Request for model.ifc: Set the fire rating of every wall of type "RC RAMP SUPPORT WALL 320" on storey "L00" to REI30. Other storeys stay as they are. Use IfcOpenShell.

First a look at what the model holds.

```python
import ifcopenshell
import ifcopenshell.util.element

model = ifcopenshell.open("model.ifc")
print(model.schema)
storey = next(s for s in model.by_type("IfcBuildingStorey") if s.Name == "L00")
walls = [e for e in ifcopenshell.util.element.get_decomposition(storey) if e.is_a("IfcWall")]
seen = {}
for e in walls:
    element_type = ifcopenshell.util.element.get_type(e)
    key = (element_type.Name if element_type != e and element_type else None, ifcopenshell.util.element.get_pset(e, "Pset_WallCommon", "FireRating"))
    seen[key] = seen.get(key, 0) + 1
for (name, value), count in sorted(seen.items(), key=str):
    print(count, "x", name, "|", value)
```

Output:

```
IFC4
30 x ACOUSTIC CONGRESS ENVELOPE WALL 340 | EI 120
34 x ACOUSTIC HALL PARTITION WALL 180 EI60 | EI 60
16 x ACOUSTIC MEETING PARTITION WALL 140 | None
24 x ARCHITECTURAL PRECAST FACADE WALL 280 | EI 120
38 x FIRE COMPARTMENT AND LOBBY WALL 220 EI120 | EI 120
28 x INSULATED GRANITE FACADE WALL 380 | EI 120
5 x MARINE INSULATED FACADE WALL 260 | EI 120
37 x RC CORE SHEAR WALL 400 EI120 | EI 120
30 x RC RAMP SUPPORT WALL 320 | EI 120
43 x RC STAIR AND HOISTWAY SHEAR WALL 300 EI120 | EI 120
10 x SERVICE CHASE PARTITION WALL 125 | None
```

```python
import ifcopenshell
import ifcopenshell.api.pset
import ifcopenshell.util.element

model = ifcopenshell.open("model.ifc")

storey = next(s for s in model.by_type("IfcBuildingStorey") if s.Name == "L00")
walls = [e for e in ifcopenshell.util.element.get_decomposition(storey) if e.is_a("IfcWall")]

count = 0
for e in walls:
    element_type = ifcopenshell.util.element.get_type(e)
    if element_type in (None, e) or element_type.Name != "RC RAMP SUPPORT WALL 320":
        continue
    # add_pset returns the element's existing set when there is one.
    pset = ifcopenshell.api.pset.add_pset(model, product=e, name="Pset_WallCommon")
    ifcopenshell.api.pset.edit_pset(model, pset=pset, properties={"FireRating": "REI30"})
    count += 1

print(count, "walls updated")

model.write("model_updated.ifc")
```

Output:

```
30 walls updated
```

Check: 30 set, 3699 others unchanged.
